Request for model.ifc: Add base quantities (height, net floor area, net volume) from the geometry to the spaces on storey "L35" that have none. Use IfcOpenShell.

First a look at what the model holds.

```python
import ifcopenshell
import ifcopenshell.util.element
import ifcopenshell.util.unit

model = ifcopenshell.open("model.ifc")
print(model.schema)
for unit_type in ("LENGTHUNIT", "AREAUNIT", "VOLUMEUNIT"):
    print(unit_type, ifcopenshell.util.unit.calculate_unit_scale(model, unit_type))
storey = next(s for s in model.by_type("IfcBuildingStorey") if s.Name == "L35")
spaces = [e for e in ifcopenshell.util.element.get_decomposition(storey) if e.is_a("IfcSpace")]
for e in sorted(spaces, key=lambda e: e.id()):
    print(e.id(), e.is_a(), e.Name, list(ifcopenshell.util.element.get_psets(e, qtos_only=True)), sep=" | ")
```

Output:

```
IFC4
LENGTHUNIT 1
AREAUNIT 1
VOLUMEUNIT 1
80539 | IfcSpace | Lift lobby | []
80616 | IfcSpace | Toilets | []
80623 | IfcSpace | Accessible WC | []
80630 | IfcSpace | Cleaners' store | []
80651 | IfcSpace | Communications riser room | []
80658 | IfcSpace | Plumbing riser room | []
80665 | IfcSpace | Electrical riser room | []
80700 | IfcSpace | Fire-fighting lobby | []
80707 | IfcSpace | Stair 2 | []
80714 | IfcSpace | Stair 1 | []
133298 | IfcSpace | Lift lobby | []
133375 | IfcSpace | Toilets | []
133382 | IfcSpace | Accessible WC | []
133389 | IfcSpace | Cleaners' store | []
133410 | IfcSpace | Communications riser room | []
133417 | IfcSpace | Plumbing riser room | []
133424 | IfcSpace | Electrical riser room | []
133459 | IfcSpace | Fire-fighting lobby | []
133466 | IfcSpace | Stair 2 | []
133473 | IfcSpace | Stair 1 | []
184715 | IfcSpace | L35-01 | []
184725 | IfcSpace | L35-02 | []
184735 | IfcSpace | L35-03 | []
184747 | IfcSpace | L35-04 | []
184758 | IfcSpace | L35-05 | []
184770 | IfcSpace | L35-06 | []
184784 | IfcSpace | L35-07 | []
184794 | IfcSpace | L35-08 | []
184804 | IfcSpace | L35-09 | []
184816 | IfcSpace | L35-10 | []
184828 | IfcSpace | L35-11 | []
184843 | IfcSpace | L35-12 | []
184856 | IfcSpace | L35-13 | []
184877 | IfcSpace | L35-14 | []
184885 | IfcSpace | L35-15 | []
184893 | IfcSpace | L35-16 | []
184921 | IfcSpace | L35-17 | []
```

```python
import ifcopenshell
import ifcopenshell.api.pset
import ifcopenshell.geom
import ifcopenshell.util.element
import ifcopenshell.util.shape
import ifcopenshell.util.unit

model = ifcopenshell.open("model.ifc")
unit_scale = ifcopenshell.util.unit.calculate_unit_scale(model)
area_scale = ifcopenshell.util.unit.calculate_unit_scale(model, "AREAUNIT")
volume_scale = ifcopenshell.util.unit.calculate_unit_scale(model, "VOLUMEUNIT")
settings = ifcopenshell.geom.settings()

storey = next(s for s in model.by_type("IfcBuildingStorey") if s.Name == "L35")
spaces = [e for e in ifcopenshell.util.element.get_decomposition(storey) if e.is_a("IfcSpace")]

for e in sorted(spaces, key=lambda e: e.id()):
    if ifcopenshell.util.element.get_psets(e, qtos_only=True, should_inherit=False):
        continue
    # Geometry comes back in metres, in the element's own axes.
    shape = ifcopenshell.geom.create_shape(settings, e)
    values = {
        "Height": ifcopenshell.util.shape.get_z(shape.geometry) / unit_scale,
        "NetFloorArea": ifcopenshell.util.shape.get_footprint_area(shape.geometry) / area_scale,
        "NetVolume": ifcopenshell.util.shape.get_volume(shape.geometry) / volume_scale,
    }
    qto = ifcopenshell.api.pset.add_qto(model, product=e, name="Qto_SpaceBaseQuantities")
    ifcopenshell.api.pset.edit_qto(model, qto=qto, properties=values)
    print(e.id(), {k: round(v, 3) for k, v in values.items()})

model.write("model_v2.ifc")
```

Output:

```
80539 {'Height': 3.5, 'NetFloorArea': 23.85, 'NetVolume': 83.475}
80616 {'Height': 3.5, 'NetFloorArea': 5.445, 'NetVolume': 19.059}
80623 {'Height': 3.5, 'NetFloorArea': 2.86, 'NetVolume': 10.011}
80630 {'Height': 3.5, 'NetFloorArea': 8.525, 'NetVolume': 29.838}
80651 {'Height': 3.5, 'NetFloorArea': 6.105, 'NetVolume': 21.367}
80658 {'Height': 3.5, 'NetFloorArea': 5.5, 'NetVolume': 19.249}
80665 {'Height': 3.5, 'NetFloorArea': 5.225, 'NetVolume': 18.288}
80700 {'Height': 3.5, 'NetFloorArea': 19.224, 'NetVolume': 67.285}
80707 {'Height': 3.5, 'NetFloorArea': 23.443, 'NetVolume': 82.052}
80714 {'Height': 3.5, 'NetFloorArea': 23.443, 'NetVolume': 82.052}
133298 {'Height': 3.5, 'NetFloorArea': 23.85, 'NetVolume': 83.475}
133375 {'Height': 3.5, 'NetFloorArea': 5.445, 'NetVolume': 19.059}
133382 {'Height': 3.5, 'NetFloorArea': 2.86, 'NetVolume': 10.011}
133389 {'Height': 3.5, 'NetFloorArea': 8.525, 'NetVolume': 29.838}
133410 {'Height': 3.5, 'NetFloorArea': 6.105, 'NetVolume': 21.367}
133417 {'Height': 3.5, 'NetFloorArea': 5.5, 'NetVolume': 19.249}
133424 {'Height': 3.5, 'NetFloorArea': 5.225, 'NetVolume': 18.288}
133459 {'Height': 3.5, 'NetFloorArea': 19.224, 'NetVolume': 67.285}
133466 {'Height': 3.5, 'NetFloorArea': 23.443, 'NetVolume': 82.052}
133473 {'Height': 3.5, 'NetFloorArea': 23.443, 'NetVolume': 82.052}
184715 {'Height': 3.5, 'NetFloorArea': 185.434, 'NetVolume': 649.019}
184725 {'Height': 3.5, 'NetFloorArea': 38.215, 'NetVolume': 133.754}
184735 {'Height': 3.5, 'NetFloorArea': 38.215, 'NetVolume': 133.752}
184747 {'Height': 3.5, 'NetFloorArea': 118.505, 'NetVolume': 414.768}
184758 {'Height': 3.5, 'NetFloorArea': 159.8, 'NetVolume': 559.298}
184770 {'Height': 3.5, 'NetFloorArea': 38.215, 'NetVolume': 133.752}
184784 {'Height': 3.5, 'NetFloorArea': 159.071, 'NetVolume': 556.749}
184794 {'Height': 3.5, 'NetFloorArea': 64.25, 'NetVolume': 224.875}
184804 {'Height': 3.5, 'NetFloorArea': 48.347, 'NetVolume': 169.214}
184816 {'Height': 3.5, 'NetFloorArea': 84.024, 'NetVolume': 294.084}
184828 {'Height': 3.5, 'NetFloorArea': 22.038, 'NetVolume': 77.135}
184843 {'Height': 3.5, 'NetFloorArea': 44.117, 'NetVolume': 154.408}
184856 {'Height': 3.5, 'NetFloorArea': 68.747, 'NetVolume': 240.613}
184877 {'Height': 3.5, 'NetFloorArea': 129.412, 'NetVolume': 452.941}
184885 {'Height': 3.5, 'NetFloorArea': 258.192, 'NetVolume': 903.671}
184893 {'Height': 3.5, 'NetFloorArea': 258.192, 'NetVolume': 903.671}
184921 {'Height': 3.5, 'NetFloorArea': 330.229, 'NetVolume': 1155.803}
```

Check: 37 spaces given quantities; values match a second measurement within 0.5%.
